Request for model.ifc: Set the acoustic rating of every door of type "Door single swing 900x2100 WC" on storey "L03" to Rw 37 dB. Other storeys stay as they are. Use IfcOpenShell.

First a look at what the model holds.

```python
import ifcopenshell
import ifcopenshell.util.element

model = ifcopenshell.open("model.ifc")
print(model.schema)
storey = next(s for s in model.by_type("IfcBuildingStorey") if s.Name == "L03")
doors = [e for e in ifcopenshell.util.element.get_decomposition(storey) if e.is_a("IfcDoor")]
seen = {}
for e in doors:
    element_type = ifcopenshell.util.element.get_type(e)
    key = (element_type.Name if element_type != e and element_type else None, ifcopenshell.util.element.get_pset(e, "Pset_DoorCommon", "AcousticRating"))
    seen[key] = seen.get(key, 0) + 1
for (name, value), count in sorted(seen.items(), key=str):
    print(count, "x", name, "|", value)
```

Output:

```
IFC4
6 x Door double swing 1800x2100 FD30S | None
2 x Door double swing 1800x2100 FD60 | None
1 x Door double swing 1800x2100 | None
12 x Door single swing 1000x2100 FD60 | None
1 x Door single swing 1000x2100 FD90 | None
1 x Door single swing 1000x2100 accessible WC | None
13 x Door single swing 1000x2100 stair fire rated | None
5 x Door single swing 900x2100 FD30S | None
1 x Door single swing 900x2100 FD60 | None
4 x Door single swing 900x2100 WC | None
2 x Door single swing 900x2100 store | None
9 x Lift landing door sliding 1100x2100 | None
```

```python
import ifcopenshell
import ifcopenshell.api.pset
import ifcopenshell.util.element

model = ifcopenshell.open("model.ifc")

storey = next(s for s in model.by_type("IfcBuildingStorey") if s.Name == "L03")
doors = [e for e in ifcopenshell.util.element.get_decomposition(storey) if e.is_a("IfcDoor")]

count = 0
for e in doors:
    element_type = ifcopenshell.util.element.get_type(e)
    if element_type in (None, e) or element_type.Name != "Door single swing 900x2100 WC":
        continue
    # add_pset returns the element's existing set when there is one.
    pset = ifcopenshell.api.pset.add_pset(model, product=e, name="Pset_DoorCommon")
    ifcopenshell.api.pset.edit_pset(model, pset=pset, properties={"AcousticRating": "Rw 37 dB"})
    count += 1

print(count, "doors updated")

model.write("model_updated.ifc")
```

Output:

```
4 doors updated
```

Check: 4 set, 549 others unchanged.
